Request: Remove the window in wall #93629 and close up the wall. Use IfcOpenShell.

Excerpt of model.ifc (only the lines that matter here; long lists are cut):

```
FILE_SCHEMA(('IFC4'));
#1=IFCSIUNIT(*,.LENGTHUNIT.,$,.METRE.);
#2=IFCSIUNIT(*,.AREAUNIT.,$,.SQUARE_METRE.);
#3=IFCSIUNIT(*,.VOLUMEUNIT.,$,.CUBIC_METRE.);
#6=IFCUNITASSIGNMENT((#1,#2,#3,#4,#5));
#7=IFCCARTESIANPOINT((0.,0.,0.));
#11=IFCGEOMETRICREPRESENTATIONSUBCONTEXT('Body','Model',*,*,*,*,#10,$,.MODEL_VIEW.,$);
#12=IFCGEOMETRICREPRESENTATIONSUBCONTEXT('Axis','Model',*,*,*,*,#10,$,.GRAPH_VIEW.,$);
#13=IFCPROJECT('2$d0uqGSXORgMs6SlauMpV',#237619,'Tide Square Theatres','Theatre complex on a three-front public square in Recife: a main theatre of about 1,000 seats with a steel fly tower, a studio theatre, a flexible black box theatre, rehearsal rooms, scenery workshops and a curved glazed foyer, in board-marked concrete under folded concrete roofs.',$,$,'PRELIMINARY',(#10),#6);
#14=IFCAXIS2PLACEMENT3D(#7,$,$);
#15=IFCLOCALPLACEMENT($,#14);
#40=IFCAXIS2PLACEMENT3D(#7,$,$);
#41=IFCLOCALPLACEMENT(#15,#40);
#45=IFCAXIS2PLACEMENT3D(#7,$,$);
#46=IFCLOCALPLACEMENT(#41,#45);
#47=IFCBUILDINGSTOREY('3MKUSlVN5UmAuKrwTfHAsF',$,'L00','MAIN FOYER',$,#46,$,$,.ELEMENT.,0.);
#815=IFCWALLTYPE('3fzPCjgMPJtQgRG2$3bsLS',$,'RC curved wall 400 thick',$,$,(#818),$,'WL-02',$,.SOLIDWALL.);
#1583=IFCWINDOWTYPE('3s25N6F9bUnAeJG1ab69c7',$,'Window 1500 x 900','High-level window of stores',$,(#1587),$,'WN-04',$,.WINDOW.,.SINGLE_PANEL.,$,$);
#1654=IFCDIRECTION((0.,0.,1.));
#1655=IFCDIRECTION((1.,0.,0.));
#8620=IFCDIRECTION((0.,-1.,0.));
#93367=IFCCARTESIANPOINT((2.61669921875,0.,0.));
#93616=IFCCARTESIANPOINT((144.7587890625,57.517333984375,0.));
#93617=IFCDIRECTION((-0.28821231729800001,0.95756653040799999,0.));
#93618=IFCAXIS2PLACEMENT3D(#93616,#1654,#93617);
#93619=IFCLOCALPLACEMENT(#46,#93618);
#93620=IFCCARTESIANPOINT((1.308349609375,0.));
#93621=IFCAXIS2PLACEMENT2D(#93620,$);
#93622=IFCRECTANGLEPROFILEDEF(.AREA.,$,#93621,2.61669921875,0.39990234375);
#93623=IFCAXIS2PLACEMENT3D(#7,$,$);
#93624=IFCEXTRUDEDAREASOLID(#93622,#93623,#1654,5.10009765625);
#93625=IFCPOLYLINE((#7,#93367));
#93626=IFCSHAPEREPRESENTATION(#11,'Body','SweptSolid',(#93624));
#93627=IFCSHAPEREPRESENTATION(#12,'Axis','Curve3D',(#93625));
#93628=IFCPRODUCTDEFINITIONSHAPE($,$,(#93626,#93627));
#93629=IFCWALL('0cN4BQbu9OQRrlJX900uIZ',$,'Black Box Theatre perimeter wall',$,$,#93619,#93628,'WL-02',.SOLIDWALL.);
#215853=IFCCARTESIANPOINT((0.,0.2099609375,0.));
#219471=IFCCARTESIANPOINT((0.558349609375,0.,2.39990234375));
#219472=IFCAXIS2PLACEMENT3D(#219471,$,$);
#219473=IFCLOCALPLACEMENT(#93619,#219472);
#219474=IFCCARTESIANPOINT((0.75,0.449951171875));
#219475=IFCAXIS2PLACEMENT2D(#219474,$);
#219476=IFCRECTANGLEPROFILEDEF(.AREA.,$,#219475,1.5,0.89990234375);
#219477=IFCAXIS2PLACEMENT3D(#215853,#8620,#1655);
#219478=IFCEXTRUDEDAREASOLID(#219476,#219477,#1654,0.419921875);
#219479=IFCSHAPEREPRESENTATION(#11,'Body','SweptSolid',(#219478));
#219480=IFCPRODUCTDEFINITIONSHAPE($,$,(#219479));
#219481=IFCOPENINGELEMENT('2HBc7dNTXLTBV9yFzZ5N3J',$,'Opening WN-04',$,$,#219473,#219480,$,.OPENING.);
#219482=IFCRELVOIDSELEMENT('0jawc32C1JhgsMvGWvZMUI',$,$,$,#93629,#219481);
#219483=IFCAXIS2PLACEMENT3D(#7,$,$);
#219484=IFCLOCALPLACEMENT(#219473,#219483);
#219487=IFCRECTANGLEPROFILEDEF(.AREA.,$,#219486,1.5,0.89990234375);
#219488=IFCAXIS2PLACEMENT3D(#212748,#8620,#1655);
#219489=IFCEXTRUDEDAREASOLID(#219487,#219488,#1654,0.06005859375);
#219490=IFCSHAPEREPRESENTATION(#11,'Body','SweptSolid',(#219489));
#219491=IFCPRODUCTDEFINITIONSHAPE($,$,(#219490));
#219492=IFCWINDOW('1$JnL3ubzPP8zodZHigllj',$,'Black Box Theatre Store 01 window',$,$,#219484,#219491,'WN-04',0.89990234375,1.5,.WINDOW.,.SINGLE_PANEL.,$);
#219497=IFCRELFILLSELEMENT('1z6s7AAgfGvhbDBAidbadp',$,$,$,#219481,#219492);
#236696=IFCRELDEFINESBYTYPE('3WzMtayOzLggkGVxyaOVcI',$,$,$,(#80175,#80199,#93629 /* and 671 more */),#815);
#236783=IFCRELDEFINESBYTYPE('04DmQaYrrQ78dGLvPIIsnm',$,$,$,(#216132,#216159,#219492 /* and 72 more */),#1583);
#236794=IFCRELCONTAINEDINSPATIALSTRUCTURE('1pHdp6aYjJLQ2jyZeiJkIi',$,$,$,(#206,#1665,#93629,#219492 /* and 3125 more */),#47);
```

```python
import ifcopenshell
import ifcopenshell.api.feature
import ifcopenshell.api.root
import ifcopenshell.geom
import ifcopenshell.util.shape

model = ifcopenshell.open("model.ifc")
settings = ifcopenshell.geom.settings()


def volume(element):
    """Net volume in cubic metres, openings subtracted."""
    shape = ifcopenshell.geom.create_shape(settings, element)
    return ifcopenshell.util.shape.get_volume(shape.geometry)


window = model.by_id(219492)
opening = window.FillsVoids[0].RelatingOpeningElement
wall = opening.VoidsElements[0].RelatingBuildingElement
before = volume(wall)

ifcopenshell.api.root.remove_product(model, product=window)
ifcopenshell.api.feature.remove_feature(model, feature=opening)

after = volume(wall)

print(f"wall volume {before:.3f} -> {after:.3f} m3")

model.write("model_edited.ifc")
```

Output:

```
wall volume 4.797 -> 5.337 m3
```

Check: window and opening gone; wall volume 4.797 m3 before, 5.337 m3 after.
